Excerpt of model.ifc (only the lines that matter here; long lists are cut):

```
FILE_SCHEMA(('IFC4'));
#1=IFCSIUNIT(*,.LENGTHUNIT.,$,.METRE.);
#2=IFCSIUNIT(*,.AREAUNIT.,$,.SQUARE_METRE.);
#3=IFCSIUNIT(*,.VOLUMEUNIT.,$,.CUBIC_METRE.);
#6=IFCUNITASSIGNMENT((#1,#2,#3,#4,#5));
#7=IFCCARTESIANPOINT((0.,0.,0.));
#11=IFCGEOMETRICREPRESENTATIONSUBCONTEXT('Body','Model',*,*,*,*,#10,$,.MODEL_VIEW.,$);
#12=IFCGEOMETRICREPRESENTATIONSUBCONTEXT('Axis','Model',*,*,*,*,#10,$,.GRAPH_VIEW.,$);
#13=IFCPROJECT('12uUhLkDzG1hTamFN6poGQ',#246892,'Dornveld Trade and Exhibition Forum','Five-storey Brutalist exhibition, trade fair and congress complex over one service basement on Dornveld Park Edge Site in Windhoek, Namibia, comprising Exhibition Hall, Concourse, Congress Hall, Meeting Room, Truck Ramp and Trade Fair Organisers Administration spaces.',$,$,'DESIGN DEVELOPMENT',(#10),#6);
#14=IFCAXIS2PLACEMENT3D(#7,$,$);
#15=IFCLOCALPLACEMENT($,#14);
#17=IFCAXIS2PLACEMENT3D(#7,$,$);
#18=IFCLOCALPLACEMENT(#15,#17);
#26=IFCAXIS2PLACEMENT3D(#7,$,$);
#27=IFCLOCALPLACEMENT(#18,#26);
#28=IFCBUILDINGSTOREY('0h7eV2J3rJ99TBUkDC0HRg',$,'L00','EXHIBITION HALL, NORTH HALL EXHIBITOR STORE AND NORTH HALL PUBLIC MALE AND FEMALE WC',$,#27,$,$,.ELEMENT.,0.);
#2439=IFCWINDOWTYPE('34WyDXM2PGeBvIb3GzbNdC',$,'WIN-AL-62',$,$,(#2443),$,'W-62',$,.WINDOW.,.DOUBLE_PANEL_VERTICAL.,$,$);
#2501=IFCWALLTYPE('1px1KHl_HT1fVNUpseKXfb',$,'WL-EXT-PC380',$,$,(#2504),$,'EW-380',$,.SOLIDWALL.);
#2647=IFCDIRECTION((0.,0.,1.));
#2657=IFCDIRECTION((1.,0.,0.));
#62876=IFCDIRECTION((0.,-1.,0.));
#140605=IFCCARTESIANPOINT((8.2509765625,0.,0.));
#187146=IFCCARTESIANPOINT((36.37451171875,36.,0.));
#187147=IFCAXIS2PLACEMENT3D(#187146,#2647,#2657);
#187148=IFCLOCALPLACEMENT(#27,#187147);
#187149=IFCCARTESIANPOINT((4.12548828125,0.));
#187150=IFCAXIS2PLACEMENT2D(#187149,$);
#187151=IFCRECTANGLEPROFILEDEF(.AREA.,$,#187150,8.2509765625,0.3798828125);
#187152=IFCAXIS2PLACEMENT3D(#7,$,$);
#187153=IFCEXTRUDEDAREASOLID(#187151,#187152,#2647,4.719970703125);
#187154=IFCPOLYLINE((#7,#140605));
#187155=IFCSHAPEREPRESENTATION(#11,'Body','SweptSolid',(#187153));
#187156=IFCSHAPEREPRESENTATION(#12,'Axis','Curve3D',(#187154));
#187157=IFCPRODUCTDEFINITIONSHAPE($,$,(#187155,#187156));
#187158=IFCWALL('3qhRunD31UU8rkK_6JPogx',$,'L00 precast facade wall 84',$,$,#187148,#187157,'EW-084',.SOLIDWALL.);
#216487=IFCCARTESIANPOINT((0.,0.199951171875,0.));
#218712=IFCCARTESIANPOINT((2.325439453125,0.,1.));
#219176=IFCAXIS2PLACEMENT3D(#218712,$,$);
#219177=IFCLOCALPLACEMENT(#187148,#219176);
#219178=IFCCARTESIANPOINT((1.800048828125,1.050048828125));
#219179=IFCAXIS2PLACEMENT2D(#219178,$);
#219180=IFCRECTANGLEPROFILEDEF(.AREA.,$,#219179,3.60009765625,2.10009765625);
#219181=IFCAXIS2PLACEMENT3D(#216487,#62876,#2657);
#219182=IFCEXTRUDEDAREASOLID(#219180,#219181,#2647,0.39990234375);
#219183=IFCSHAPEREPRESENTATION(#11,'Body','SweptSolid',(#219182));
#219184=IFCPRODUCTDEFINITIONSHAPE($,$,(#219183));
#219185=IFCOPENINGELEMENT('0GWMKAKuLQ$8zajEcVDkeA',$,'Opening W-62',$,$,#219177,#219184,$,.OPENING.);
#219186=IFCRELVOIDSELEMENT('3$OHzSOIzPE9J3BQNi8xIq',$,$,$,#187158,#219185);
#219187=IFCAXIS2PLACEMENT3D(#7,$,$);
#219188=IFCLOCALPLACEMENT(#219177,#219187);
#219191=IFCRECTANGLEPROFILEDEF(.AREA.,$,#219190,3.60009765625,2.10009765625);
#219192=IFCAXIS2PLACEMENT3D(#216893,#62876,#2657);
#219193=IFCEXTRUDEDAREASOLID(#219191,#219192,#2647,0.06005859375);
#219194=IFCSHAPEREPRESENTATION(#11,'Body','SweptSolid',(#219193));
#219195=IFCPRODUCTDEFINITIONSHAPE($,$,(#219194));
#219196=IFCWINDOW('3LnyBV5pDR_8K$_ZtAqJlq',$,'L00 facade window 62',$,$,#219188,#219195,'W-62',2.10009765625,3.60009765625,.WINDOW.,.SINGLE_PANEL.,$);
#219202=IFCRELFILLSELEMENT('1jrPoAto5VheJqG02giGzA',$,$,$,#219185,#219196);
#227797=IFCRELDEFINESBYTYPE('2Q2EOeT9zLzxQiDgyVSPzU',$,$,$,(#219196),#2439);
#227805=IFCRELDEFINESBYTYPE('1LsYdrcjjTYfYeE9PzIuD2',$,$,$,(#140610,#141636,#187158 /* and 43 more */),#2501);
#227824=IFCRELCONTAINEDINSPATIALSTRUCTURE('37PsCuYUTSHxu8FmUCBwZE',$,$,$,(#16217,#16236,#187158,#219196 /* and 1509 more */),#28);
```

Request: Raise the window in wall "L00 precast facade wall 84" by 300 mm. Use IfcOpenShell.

```python
import numpy as np
import ifcopenshell
import ifcopenshell.api.geometry
import ifcopenshell.util.placement
import ifcopenshell.util.unit

model = ifcopenshell.open("model.ifc")
unit_scale = ifcopenshell.util.unit.calculate_unit_scale(model)

window = model.by_id(219196)
opening = window.FillsVoids[0].RelatingOpeningElement
dz = 0.3

shift = np.array([0.0, 0.0, dz])
# The window is placed relative to its opening, so it follows when the opening moves.
matrix = ifcopenshell.util.placement.get_local_placement(opening.ObjectPlacement)
matrix[:3, 3] += shift
ifcopenshell.api.geometry.edit_object_placement(
    model, product=opening, matrix=matrix, is_si=False, should_transform_children=True
)

print(f"moved by {dz * unit_scale:+.3f} m")

model.write("model-out.ifc")
```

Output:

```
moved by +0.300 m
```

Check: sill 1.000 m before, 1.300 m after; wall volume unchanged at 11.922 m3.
